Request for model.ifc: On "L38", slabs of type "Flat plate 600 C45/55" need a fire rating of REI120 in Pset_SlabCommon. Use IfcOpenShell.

First a look at what the model holds.

```python
import ifcopenshell
import ifcopenshell.util.element

model = ifcopenshell.open("model.ifc")
print(model.schema)
storey = next(s for s in model.by_type("IfcBuildingStorey") if s.Name == "L38")
slabs = [e for e in ifcopenshell.util.element.get_decomposition(storey) if e.is_a("IfcSlab")]
seen = {}
for e in slabs:
    element_type = ifcopenshell.util.element.get_type(e)
    key = (element_type.Name if element_type != e and element_type else None, ifcopenshell.util.element.get_pset(e, "Pset_SlabCommon", "FireRating"))
    seen[key] = seen.get(key, 0) + 1
for (name, value), count in sorted(seen.items(), key=str):
    print(count, "x", name, "|", value)
```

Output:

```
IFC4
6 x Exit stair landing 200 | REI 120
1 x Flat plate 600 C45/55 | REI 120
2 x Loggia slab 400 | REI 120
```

```python
import ifcopenshell
import ifcopenshell.api.pset
import ifcopenshell.util.element

model = ifcopenshell.open("model.ifc")

storey = next(s for s in model.by_type("IfcBuildingStorey") if s.Name == "L38")
slabs = [e for e in ifcopenshell.util.element.get_decomposition(storey) if e.is_a("IfcSlab")]

count = 0
for e in slabs:
    element_type = ifcopenshell.util.element.get_type(e)
    if element_type in (None, e) or element_type.Name != "Flat plate 600 C45/55":
        continue
    found = ifcopenshell.util.element.get_pset(e, "Pset_SlabCommon", should_inherit=False)
    if found:
        pset = model.by_id(found["id"])
        if len(ifcopenshell.util.element.get_elements_by_pset(pset)) > 1:
            pset = ifcopenshell.api.pset.unshare_pset(model, products=[e], pset=pset)[0]
    else:
        pset = ifcopenshell.api.pset.add_pset(model, product=e, name="Pset_SlabCommon")
    ifcopenshell.api.pset.edit_pset(model, pset=pset, properties={"FireRating": "REI120"})
    count += 1

print(count, "slabs updated")

model.write("model_rev.ifc")
```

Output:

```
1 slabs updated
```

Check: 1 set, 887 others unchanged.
